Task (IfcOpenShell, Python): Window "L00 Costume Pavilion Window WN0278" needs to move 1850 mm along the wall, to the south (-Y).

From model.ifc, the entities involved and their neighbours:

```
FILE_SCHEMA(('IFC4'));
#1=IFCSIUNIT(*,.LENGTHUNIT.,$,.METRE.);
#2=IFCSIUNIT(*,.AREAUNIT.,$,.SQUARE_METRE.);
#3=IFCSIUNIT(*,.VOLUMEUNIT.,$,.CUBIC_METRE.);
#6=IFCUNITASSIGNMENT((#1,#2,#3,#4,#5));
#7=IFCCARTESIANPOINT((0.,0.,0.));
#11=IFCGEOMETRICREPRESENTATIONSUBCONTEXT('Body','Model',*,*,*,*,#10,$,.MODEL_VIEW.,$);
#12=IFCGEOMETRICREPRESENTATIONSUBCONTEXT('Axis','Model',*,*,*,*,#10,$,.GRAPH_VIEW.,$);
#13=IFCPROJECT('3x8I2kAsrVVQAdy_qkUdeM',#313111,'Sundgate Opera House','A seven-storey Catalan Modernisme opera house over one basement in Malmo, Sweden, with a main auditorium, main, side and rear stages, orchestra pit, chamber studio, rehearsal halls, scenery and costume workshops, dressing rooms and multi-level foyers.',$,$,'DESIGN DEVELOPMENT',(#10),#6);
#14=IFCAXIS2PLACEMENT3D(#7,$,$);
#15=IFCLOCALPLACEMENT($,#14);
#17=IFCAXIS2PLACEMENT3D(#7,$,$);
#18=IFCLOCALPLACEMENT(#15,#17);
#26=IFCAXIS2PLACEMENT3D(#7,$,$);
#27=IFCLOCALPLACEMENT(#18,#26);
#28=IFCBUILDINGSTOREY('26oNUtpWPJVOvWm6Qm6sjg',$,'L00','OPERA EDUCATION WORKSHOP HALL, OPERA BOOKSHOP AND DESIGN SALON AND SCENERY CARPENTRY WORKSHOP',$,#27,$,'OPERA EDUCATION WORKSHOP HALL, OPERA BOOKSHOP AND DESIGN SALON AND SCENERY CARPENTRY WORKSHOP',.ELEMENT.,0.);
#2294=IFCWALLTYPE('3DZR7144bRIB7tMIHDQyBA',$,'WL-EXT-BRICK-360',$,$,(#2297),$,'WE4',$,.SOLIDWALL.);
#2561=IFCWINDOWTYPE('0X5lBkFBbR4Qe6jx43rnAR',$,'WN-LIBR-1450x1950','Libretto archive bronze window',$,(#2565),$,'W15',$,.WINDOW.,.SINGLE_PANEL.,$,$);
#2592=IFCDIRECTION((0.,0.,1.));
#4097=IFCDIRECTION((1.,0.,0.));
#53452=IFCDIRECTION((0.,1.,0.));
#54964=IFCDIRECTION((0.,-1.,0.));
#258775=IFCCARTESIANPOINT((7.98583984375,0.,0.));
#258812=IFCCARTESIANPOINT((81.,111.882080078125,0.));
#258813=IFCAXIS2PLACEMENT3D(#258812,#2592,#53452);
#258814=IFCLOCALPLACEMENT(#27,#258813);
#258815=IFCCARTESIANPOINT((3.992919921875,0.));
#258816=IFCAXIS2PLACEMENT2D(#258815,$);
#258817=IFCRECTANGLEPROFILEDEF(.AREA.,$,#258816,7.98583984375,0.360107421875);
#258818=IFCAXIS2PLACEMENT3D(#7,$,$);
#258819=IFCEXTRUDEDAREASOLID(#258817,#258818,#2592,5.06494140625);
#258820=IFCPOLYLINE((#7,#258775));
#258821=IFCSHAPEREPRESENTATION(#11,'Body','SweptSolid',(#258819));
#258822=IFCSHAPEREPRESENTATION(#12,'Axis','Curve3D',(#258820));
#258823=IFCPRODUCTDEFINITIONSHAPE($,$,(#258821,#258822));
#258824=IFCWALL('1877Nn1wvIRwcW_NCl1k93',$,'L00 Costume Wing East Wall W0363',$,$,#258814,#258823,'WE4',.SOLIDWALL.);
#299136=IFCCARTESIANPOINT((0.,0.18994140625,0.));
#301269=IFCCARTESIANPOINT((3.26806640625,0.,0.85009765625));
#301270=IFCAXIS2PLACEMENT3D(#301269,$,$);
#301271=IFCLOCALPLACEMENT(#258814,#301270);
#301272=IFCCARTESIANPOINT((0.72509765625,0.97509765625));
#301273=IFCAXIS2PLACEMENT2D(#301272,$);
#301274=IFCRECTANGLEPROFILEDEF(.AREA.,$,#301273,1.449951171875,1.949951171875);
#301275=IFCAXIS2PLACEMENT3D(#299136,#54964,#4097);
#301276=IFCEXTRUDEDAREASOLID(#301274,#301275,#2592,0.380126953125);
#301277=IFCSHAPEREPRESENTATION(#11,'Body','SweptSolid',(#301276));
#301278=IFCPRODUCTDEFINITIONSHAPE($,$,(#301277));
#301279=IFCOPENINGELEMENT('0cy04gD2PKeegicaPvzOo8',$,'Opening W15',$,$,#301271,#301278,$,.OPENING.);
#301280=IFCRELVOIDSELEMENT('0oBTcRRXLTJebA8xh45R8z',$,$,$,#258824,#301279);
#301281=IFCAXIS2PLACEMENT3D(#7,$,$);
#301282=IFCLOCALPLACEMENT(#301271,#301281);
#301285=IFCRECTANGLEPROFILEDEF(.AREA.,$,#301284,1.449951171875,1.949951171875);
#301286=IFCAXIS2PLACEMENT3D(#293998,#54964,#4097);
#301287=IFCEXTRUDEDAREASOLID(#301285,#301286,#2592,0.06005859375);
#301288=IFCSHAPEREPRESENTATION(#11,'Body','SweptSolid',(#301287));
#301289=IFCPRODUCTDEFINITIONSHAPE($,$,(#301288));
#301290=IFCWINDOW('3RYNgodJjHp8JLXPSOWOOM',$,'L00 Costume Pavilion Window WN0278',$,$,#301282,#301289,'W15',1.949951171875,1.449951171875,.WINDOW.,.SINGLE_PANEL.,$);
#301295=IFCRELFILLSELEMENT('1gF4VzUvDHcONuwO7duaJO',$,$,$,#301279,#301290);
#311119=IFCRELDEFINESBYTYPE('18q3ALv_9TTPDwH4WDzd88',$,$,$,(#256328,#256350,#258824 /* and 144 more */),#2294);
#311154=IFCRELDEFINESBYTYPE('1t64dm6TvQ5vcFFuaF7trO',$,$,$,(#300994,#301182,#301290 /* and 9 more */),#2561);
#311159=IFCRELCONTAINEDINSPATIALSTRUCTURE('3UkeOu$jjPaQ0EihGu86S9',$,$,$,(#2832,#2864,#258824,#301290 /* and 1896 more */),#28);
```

```python
import ifcopenshell
import ifcopenshell.api.geometry
import ifcopenshell.util.placement

model = ifcopenshell.open("model.ifc")

window = model.by_guid("3RYNgodJjHp8JLXPSOWOOM")
opening = window.FillsVoids[0].RelatingOpeningElement
wall = opening.VoidsElements[0].RelatingBuildingElement

wall_matrix = ifcopenshell.util.placement.get_local_placement(wall.ObjectPlacement)
shift = wall_matrix[:3, 0] * -1.85
before = ifcopenshell.util.placement.get_local_placement(window.ObjectPlacement)[:3, 3].copy()

# The window is placed relative to its opening, so it follows when the opening moves.
matrix = ifcopenshell.util.placement.get_local_placement(opening.ObjectPlacement)
matrix[:3, 3] += shift
ifcopenshell.api.geometry.edit_object_placement(
    model, product=opening, matrix=matrix, is_si=False, should_transform_children=True
)

after = ifcopenshell.util.placement.get_local_placement(window.ObjectPlacement)[:3, 3]
print("window moved by", (after - before).round(3) + 0.0)

model.write("model_updated.ifc")
```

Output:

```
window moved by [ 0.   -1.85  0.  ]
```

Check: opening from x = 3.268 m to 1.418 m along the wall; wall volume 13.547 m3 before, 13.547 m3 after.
